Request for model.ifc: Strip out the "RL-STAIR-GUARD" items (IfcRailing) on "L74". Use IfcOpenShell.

First a look at what the model holds.

```python
import ifcopenshell
import ifcopenshell.util.element

model = ifcopenshell.open("model.ifc")
print(model.schema)
storey = next(s for s in model.by_type("IfcBuildingStorey") if s.Name == "L74")
railings = [e for e in ifcopenshell.util.element.get_decomposition(storey) if e.is_a("IfcRailing")]
seen = {}
for e in railings:
    element_type = ifcopenshell.util.element.get_type(e)
    name = element_type.Name if element_type not in (None, e) else None
    seen[name] = seen.get(name, 0) + 1
for name, count in sorted(seen.items(), key=str):
    print(count, "x", name)
```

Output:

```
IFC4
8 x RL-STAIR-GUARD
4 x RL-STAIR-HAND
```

```python
import ifcopenshell
import ifcopenshell.api.root
import ifcopenshell.util.element

model = ifcopenshell.open("model.ifc")

storey = next(s for s in model.by_type("IfcBuildingStorey") if s.Name == "L74")
railings = [e for e in ifcopenshell.util.element.get_decomposition(storey) if e.is_a("IfcRailing")]
targets = [e for e in railings if (t := ifcopenshell.util.element.get_type(e)) not in (None, e) and t.Name == "RL-STAIR-GUARD"]

for e in targets:
    ifcopenshell.api.root.remove_product(model, product=e)
print(len(targets), "removed")

model.write("model_rev.ifc")
```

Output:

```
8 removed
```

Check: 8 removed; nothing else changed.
